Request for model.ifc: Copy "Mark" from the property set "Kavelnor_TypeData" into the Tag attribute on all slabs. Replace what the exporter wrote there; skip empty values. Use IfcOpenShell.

First a look at what the model holds.

```python
import ifcopenshell
import ifcopenshell.util.element

model = ifcopenshell.open("model.ifc")
print(model.schema)
slabs = model.by_type("IfcSlab")
print(len(slabs), "slabs")
for e in slabs[:8]:
    source = ifcopenshell.util.element.get_pset(e, "Kavelnor_TypeData", "Mark")
    target = e.Tag
    print(e.id(), repr(source), repr(target), sep=" | ")
```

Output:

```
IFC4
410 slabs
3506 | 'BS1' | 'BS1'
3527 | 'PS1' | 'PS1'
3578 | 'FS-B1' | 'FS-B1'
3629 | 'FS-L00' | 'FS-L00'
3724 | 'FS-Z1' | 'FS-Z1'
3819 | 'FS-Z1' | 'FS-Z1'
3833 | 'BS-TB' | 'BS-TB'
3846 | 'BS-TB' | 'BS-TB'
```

```python
import ifcopenshell
import ifcopenshell.util.element

model = ifcopenshell.open("model.ifc")

count = 0
for e in model.by_type("IfcSlab"):
    value = ifcopenshell.util.element.get_pset(e, "Kavelnor_TypeData", "Mark")
    current = e.Tag
    if not value or not value.strip() or current == value:
        continue
    e.Tag = value
    count += 1

print(count, "slabs updated")

model.write("model_updated.ifc")
```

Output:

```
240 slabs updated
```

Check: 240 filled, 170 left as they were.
